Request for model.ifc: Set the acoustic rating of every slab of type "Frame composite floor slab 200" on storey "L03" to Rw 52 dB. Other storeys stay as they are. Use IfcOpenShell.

First a look at what the model holds.

```python
import ifcopenshell
import ifcopenshell.util.element

model = ifcopenshell.open("model.ifc")
print(model.schema)
storey = next(s for s in model.by_type("IfcBuildingStorey") if s.Name == "L03")
slabs = [e for e in ifcopenshell.util.element.get_decomposition(storey) if e.is_a("IfcSlab")]
seen = {}
for e in slabs:
    element_type = ifcopenshell.util.element.get_type(e)
    key = (element_type.Name if element_type != e and element_type else None, ifcopenshell.util.element.get_pset(e, "Pset_SlabCommon", "AcousticRating"))
    seen[key] = seen.get(key, 0) + 1
for (name, value), count in sorted(seen.items(), key=str):
    print(count, "x", name, "|", value)
```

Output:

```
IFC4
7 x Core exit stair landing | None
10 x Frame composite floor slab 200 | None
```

```python
import ifcopenshell
import ifcopenshell.api.pset
import ifcopenshell.util.element

model = ifcopenshell.open("model.ifc")

storey = next(s for s in model.by_type("IfcBuildingStorey") if s.Name == "L03")
slabs = [e for e in ifcopenshell.util.element.get_decomposition(storey) if e.is_a("IfcSlab")]

count = 0
for e in slabs:
    element_type = ifcopenshell.util.element.get_type(e)
    if element_type in (None, e) or element_type.Name != "Frame composite floor slab 200":
        continue
    found = ifcopenshell.util.element.get_pset(e, "Pset_SlabCommon", should_inherit=False)
    if found:
        pset = model.by_id(found["id"])
        if len(ifcopenshell.util.element.get_elements_by_pset(pset)) > 1:
            pset = ifcopenshell.api.pset.unshare_pset(model, products=[e], pset=pset)[0]
    else:
        pset = ifcopenshell.api.pset.add_pset(model, product=e, name="Pset_SlabCommon")
    ifcopenshell.api.pset.edit_pset(model, pset=pset, properties={"AcousticRating": "Rw 52 dB"})
    count += 1

print(count, "slabs updated")

model.write("model_rev.ifc")
```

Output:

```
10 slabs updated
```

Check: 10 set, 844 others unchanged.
